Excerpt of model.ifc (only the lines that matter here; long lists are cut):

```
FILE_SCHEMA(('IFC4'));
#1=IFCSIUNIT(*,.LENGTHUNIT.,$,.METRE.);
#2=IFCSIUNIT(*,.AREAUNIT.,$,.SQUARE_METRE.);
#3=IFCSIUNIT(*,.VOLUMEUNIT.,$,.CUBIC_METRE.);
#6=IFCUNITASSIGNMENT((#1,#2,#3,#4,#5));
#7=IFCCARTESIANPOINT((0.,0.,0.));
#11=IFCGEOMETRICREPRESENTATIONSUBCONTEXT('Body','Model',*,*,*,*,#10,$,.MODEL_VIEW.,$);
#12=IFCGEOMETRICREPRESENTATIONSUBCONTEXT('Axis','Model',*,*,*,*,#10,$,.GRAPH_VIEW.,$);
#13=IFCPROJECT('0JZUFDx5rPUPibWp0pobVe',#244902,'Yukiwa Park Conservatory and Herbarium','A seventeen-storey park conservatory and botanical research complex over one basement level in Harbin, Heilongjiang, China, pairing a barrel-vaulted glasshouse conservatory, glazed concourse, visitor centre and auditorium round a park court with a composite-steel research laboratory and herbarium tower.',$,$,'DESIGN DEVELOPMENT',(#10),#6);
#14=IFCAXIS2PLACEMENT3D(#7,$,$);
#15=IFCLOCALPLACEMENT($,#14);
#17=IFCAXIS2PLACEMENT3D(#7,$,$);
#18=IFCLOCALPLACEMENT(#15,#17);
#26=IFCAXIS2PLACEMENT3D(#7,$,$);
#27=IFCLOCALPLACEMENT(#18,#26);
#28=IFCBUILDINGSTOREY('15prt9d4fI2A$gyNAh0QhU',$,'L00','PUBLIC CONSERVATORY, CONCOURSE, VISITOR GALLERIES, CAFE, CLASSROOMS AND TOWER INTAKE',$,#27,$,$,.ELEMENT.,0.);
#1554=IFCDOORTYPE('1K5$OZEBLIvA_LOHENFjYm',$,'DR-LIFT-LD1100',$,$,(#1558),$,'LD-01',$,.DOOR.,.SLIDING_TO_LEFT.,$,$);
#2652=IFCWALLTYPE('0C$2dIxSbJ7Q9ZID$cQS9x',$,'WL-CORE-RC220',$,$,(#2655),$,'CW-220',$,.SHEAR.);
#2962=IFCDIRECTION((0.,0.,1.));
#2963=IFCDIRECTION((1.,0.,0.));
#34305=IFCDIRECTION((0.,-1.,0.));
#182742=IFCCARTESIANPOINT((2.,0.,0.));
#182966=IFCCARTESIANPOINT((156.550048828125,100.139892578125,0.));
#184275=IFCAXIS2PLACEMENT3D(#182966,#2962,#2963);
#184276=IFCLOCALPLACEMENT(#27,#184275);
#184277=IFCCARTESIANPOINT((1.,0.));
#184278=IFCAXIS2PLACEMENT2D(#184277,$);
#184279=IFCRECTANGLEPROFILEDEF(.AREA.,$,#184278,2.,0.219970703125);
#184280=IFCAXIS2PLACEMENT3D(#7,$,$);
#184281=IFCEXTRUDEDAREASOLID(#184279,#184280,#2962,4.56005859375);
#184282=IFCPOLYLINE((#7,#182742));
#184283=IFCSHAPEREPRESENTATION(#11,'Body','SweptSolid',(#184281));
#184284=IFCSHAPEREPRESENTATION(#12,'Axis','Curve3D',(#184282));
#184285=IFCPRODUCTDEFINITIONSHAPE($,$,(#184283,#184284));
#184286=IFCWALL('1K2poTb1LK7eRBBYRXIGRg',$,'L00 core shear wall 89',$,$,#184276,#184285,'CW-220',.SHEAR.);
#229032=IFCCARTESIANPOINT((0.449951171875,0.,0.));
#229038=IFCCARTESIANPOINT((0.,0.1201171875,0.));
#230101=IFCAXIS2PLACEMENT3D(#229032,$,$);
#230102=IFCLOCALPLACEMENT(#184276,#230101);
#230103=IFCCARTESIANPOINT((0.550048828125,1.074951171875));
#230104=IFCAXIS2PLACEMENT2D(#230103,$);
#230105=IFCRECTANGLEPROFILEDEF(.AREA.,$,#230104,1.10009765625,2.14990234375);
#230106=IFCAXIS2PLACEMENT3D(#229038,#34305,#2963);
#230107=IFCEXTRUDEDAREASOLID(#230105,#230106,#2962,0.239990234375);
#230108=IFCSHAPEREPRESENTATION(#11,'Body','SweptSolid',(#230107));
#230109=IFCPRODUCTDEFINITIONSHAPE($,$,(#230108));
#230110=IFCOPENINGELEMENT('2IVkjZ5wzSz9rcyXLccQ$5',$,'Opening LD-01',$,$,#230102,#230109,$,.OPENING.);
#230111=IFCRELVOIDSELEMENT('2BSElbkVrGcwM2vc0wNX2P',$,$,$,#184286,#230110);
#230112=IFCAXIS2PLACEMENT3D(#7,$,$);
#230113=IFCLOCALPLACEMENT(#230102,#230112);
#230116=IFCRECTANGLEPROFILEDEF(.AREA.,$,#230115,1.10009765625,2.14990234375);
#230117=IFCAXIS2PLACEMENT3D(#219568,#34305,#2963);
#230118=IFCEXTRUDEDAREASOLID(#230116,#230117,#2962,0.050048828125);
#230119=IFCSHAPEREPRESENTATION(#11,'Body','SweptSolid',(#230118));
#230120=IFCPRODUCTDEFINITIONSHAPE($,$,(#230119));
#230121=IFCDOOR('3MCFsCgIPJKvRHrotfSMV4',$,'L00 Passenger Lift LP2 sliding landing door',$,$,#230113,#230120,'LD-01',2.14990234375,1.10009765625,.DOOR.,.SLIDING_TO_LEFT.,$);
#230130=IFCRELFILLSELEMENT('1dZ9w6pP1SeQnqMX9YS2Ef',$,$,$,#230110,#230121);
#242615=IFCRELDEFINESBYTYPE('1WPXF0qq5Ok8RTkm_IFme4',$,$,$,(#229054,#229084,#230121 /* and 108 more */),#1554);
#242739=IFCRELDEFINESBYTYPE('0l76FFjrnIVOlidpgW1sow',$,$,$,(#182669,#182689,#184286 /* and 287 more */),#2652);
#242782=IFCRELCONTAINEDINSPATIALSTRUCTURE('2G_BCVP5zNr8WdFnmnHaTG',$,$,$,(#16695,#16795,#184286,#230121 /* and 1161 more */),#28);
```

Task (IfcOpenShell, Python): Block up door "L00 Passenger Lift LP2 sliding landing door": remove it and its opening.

```python
import ifcopenshell
import ifcopenshell.api.feature
import ifcopenshell.api.root
import ifcopenshell.geom
import ifcopenshell.util.shape

model = ifcopenshell.open("model.ifc")
settings = ifcopenshell.geom.settings()


def volume(element):
    """Net volume in cubic metres, openings subtracted."""
    shape = ifcopenshell.geom.create_shape(settings, element)
    return ifcopenshell.util.shape.get_volume(shape.geometry)


door = model.by_id(230121)
opening = door.FillsVoids[0].RelatingOpeningElement
wall = opening.VoidsElements[0].RelatingBuildingElement
before = volume(wall)

ifcopenshell.api.root.remove_product(model, product=door)
ifcopenshell.api.feature.remove_feature(model, feature=opening)

after = volume(wall)

print(f"wall volume {before:.3f} -> {after:.3f} m3")

model.write("model_edited.ifc")
```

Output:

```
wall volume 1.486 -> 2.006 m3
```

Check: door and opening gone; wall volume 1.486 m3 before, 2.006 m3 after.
